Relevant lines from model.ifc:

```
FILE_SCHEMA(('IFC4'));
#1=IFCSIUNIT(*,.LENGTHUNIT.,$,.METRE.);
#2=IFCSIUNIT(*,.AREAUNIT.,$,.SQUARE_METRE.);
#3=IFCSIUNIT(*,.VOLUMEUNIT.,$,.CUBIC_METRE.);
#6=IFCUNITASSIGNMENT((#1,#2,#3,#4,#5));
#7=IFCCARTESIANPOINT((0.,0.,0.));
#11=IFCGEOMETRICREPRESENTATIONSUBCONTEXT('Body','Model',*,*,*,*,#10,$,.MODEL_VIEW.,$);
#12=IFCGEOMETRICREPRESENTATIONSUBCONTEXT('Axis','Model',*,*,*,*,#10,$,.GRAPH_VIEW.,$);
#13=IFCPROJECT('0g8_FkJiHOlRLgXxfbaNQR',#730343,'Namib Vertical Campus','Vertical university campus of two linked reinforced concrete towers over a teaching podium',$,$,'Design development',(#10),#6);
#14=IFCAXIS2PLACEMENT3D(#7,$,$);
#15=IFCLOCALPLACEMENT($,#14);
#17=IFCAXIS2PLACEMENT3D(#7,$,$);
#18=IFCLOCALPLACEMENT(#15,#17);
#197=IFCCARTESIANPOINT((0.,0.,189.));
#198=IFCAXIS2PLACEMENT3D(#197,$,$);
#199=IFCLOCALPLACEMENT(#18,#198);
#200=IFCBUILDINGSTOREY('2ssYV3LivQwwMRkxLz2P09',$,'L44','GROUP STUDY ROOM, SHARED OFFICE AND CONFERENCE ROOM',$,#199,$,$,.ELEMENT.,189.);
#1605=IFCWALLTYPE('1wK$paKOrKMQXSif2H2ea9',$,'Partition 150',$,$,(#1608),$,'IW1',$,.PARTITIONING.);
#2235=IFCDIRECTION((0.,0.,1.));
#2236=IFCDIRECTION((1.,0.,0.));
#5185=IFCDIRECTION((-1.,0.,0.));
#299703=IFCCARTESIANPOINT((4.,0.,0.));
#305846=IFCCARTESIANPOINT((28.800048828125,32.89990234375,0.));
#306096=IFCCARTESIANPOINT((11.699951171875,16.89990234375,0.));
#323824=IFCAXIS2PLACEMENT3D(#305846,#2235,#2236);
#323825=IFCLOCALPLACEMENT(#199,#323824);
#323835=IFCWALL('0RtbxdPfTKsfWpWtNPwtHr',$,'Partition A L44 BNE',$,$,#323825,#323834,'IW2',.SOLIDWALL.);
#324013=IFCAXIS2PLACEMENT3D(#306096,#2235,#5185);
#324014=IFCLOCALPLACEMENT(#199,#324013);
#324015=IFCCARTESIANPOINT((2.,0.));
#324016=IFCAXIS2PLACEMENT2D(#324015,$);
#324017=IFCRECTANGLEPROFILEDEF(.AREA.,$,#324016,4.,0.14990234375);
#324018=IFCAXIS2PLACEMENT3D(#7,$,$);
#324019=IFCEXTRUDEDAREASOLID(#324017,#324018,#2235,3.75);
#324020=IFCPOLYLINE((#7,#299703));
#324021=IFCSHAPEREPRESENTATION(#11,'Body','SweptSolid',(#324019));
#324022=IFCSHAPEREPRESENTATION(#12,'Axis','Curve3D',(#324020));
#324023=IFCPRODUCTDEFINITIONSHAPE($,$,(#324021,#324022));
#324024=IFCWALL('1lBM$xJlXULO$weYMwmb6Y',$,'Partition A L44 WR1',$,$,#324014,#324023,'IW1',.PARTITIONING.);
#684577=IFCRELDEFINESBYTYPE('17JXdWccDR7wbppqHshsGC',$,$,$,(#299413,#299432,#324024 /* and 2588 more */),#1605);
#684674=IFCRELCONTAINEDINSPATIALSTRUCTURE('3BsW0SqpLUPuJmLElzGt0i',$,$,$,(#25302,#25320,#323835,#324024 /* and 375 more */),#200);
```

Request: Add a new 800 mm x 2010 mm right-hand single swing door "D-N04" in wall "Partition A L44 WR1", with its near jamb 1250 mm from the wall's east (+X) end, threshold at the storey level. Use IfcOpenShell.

```python
import numpy as np
import ifcopenshell
import ifcopenshell.api.feature
import ifcopenshell.api.geometry
import ifcopenshell.api.root
import ifcopenshell.api.spatial
import ifcopenshell.geom
import ifcopenshell.util.element
import ifcopenshell.util.placement
import ifcopenshell.util.representation
import ifcopenshell.util.shape
import ifcopenshell.util.unit

model = ifcopenshell.open("model.ifc")
unit_scale = ifcopenshell.util.unit.calculate_unit_scale(model)
settings = ifcopenshell.geom.settings()


def volume(element):
    """Net volume in cubic metres, openings subtracted."""
    shape = ifcopenshell.geom.create_shape(settings, element)
    return ifcopenshell.util.shape.get_volume(shape.geometry)


wall = model.by_guid("1lBM$xJlXULO$weYMwmb6Y")
storey = ifcopenshell.util.element.get_container(wall, ifc_class="IfcBuildingStorey")
context = ifcopenshell.util.representation.get_context(model, "Model", "Body", "MODEL_VIEW")
before = volume(wall)

width, height, from_end, sill = 0.8, 2.01, 1.25, 0.0  # metres

# The wall runs along its own X axis, and the end named is its -X end.
wall_shape = ifcopenshell.geom.create_shape(settings, wall)
x, y, z = ifcopenshell.util.shape.get_vertices(wall_shape.geometry).T
start = x.min() + from_end
face, thickness = float(y.min()), float(y.max() - y.min())
wall_matrix = ifcopenshell.util.placement.get_local_placement(wall.ObjectPlacement)
level = ifcopenshell.util.placement.get_local_placement(storey.ObjectPlacement)[2, 3]


def in_wall(x, y):
    """Placement at x, y metres in the wall's axes, at sill height."""
    matrix = wall_matrix.copy()
    matrix[:, 3] = wall_matrix @ np.array([x / unit_scale, y / unit_scale, 0.0, 1.0])
    matrix[2, 3] = level + sill / unit_scale
    return matrix


# Opening: a box that overshoots both wall faces by 50 mm.
opening = ifcopenshell.api.root.create_entity(model, ifc_class="IfcOpeningElement", predefined_type="OPENING")
box = ifcopenshell.api.geometry.add_wall_representation(
    model, context=context, length=width, height=height, thickness=thickness + 0.1
)
ifcopenshell.api.geometry.assign_representation(model, product=opening, representation=box)
ifcopenshell.api.geometry.edit_object_placement(model, product=opening, matrix=in_wall(start, face - 0.05), is_si=False)
ifcopenshell.api.feature.add_feature(model, feature=opening, element=wall)

door = ifcopenshell.api.root.create_entity(model, ifc_class="IfcDoor", name="D-N04", predefined_type="DOOR")
door.OverallWidth, door.OverallHeight = width / unit_scale, height / unit_scale
door.OperationType = "SINGLE_SWING_RIGHT"
body = ifcopenshell.api.geometry.add_door_representation(
    model,
    context=context,
    overall_width=door.OverallWidth,
    overall_height=door.OverallHeight,
    operation_type="SINGLE_SWING_RIGHT",
    lining_properties={"LiningDepth": thickness / unit_scale, "ThresholdDepth": thickness / unit_scale},
)
ifcopenshell.api.geometry.assign_representation(model, product=door, representation=body)
ifcopenshell.api.spatial.assign_container(model, products=[door], relating_structure=storey)
ifcopenshell.api.feature.add_filling(model, opening=opening, element=door)

# The lining spans the wall, so the door starts at the wall face.
ifcopenshell.api.geometry.edit_object_placement(model, product=door, matrix=in_wall(start, face), is_si=False)

after = volume(wall)

print(f"wall volume {before:.3f} -> {after:.3f} m3")

model.write("model_rev.ifc")
```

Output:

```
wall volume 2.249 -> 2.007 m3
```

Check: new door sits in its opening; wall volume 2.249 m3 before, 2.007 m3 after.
